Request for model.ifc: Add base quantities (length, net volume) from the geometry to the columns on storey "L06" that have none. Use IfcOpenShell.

First a look at what the model holds.

```python
import ifcopenshell
import ifcopenshell.util.element
import ifcopenshell.util.unit

model = ifcopenshell.open("model.ifc")
print(model.schema)
for unit_type in ("LENGTHUNIT", "AREAUNIT", "VOLUMEUNIT"):
    print(unit_type, ifcopenshell.util.unit.calculate_unit_scale(model, unit_type))
storey = next(s for s in model.by_type("IfcBuildingStorey") if s.Name == "L06")
columns = [e for e in ifcopenshell.util.element.get_decomposition(storey) if e.is_a("IfcColumn")]
for e in sorted(columns, key=lambda e: e.id()):
    print(e.id(), e.is_a(), e.Name, list(ifcopenshell.util.element.get_psets(e, qtos_only=True)), sep=" | ")
```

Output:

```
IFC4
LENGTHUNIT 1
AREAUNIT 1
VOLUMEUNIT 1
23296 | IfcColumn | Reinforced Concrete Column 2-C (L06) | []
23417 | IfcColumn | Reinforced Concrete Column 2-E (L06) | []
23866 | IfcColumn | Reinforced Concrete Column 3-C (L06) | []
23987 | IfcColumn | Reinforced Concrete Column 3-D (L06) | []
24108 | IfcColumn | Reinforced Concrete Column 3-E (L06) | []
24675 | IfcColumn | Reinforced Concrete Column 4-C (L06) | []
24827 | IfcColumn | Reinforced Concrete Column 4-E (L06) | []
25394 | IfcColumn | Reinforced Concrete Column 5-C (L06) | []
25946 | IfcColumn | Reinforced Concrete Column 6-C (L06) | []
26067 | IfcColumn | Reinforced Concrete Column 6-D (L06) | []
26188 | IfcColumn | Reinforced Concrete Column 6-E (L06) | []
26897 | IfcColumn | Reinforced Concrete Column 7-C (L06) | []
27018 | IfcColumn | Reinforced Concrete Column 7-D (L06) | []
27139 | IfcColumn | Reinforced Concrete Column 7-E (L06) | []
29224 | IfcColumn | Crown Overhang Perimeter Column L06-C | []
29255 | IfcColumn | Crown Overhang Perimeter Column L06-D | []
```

```python
import ifcopenshell
import ifcopenshell.api.pset
import ifcopenshell.geom
import ifcopenshell.util.element
import ifcopenshell.util.shape
import ifcopenshell.util.unit

model = ifcopenshell.open("model.ifc")
unit_scale = ifcopenshell.util.unit.calculate_unit_scale(model)
volume_scale = ifcopenshell.util.unit.calculate_unit_scale(model, "VOLUMEUNIT")
settings = ifcopenshell.geom.settings()

storey = next(s for s in model.by_type("IfcBuildingStorey") if s.Name == "L06")
columns = [e for e in ifcopenshell.util.element.get_decomposition(storey) if e.is_a("IfcColumn")]

for e in sorted(columns, key=lambda e: e.id()):
    if ifcopenshell.util.element.get_psets(e, qtos_only=True, should_inherit=False):
        continue
    # Geometry comes back in metres, in the element's own axes.
    shape = ifcopenshell.geom.create_shape(settings, e)
    values = {
        "Length": ifcopenshell.util.shape.get_z(shape.geometry) / unit_scale,
        "NetVolume": ifcopenshell.util.shape.get_volume(shape.geometry) / volume_scale,
    }
    qto = ifcopenshell.api.pset.add_qto(model, product=e, name="Qto_ColumnBaseQuantities")
    ifcopenshell.api.pset.edit_qto(model, qto=qto, properties=values)
    print(e.id(), {k: round(v, 3) for k, v in values.items()})

model.write("model_updated.ifc")
```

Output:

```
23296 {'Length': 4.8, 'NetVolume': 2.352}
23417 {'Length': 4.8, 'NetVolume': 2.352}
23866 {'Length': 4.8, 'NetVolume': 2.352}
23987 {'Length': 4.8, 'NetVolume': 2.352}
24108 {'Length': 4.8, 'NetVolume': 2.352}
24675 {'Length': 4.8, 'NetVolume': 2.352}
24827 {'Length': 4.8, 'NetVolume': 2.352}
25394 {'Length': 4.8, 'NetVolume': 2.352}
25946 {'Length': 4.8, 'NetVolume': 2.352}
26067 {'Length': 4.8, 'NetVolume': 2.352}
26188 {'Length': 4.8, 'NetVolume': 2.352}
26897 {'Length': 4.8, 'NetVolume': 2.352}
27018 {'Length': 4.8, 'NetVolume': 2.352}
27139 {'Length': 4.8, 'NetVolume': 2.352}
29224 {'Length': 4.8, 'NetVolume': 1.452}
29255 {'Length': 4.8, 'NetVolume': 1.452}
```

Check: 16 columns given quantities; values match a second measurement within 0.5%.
